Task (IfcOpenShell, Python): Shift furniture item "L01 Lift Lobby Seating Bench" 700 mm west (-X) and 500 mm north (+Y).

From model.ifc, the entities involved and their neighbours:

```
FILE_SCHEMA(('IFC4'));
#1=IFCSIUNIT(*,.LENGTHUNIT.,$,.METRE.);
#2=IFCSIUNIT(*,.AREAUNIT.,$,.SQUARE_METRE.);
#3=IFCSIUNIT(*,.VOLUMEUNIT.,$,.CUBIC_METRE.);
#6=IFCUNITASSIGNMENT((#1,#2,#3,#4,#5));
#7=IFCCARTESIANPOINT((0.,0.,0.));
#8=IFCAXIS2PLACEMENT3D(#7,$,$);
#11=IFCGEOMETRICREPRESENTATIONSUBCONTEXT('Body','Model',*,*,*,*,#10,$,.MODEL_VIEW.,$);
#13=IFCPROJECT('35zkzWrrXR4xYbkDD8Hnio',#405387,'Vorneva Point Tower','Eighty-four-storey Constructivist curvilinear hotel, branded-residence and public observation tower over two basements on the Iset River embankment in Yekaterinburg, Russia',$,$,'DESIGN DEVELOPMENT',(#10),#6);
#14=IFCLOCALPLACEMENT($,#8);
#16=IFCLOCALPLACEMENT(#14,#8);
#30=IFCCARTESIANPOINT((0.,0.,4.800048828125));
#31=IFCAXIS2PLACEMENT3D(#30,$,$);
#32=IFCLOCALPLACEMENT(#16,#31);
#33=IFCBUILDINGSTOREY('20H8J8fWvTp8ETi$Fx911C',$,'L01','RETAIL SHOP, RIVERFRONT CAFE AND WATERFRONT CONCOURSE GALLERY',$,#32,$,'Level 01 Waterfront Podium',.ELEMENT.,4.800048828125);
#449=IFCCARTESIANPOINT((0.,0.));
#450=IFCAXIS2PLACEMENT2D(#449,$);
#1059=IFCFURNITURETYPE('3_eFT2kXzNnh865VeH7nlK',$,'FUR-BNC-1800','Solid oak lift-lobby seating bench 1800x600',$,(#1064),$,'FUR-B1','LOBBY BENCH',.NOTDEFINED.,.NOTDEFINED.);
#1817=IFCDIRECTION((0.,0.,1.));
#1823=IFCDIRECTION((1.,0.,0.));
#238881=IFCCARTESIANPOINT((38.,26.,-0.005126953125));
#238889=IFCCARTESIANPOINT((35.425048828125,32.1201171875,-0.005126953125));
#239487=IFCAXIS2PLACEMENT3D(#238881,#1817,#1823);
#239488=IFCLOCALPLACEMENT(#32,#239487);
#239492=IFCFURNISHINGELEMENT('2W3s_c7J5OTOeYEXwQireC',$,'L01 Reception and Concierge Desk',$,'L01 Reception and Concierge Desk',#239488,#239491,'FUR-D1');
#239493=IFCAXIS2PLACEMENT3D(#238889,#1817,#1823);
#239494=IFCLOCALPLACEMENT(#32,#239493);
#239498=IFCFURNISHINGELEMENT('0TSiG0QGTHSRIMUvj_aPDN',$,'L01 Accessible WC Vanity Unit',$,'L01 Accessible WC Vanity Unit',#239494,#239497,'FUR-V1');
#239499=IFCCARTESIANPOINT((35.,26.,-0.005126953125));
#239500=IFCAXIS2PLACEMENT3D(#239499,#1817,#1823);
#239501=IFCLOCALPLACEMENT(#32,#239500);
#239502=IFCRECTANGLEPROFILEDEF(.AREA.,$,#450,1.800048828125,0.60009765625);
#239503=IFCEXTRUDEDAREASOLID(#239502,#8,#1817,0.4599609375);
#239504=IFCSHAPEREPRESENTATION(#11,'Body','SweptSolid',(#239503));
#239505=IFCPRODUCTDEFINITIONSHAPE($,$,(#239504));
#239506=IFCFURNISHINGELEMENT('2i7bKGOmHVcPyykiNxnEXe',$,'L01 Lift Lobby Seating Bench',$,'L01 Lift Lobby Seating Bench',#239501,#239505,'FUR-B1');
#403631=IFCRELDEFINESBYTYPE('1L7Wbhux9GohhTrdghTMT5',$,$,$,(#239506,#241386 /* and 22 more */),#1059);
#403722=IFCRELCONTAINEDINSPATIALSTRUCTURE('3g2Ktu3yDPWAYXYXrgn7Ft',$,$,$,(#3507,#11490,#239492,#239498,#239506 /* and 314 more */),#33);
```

```python
import ifcopenshell
import ifcopenshell.api.geometry
import ifcopenshell.util.placement

model = ifcopenshell.open("model.ifc")

item = model.by_guid("2i7bKGOmHVcPyykiNxnEXe")
matrix = ifcopenshell.util.placement.get_local_placement(item.ObjectPlacement)
matrix[0, 3] -= 0.7
matrix[1, 3] += 0.5
ifcopenshell.api.geometry.edit_object_placement(model, product=item, matrix=matrix, is_si=False)

print(ifcopenshell.util.placement.get_local_placement(item.ObjectPlacement).round(3) + 0.0)

model.write("model-out.ifc")
```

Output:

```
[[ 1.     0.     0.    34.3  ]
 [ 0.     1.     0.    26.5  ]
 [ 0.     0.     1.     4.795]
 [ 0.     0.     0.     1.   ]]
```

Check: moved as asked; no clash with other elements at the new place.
